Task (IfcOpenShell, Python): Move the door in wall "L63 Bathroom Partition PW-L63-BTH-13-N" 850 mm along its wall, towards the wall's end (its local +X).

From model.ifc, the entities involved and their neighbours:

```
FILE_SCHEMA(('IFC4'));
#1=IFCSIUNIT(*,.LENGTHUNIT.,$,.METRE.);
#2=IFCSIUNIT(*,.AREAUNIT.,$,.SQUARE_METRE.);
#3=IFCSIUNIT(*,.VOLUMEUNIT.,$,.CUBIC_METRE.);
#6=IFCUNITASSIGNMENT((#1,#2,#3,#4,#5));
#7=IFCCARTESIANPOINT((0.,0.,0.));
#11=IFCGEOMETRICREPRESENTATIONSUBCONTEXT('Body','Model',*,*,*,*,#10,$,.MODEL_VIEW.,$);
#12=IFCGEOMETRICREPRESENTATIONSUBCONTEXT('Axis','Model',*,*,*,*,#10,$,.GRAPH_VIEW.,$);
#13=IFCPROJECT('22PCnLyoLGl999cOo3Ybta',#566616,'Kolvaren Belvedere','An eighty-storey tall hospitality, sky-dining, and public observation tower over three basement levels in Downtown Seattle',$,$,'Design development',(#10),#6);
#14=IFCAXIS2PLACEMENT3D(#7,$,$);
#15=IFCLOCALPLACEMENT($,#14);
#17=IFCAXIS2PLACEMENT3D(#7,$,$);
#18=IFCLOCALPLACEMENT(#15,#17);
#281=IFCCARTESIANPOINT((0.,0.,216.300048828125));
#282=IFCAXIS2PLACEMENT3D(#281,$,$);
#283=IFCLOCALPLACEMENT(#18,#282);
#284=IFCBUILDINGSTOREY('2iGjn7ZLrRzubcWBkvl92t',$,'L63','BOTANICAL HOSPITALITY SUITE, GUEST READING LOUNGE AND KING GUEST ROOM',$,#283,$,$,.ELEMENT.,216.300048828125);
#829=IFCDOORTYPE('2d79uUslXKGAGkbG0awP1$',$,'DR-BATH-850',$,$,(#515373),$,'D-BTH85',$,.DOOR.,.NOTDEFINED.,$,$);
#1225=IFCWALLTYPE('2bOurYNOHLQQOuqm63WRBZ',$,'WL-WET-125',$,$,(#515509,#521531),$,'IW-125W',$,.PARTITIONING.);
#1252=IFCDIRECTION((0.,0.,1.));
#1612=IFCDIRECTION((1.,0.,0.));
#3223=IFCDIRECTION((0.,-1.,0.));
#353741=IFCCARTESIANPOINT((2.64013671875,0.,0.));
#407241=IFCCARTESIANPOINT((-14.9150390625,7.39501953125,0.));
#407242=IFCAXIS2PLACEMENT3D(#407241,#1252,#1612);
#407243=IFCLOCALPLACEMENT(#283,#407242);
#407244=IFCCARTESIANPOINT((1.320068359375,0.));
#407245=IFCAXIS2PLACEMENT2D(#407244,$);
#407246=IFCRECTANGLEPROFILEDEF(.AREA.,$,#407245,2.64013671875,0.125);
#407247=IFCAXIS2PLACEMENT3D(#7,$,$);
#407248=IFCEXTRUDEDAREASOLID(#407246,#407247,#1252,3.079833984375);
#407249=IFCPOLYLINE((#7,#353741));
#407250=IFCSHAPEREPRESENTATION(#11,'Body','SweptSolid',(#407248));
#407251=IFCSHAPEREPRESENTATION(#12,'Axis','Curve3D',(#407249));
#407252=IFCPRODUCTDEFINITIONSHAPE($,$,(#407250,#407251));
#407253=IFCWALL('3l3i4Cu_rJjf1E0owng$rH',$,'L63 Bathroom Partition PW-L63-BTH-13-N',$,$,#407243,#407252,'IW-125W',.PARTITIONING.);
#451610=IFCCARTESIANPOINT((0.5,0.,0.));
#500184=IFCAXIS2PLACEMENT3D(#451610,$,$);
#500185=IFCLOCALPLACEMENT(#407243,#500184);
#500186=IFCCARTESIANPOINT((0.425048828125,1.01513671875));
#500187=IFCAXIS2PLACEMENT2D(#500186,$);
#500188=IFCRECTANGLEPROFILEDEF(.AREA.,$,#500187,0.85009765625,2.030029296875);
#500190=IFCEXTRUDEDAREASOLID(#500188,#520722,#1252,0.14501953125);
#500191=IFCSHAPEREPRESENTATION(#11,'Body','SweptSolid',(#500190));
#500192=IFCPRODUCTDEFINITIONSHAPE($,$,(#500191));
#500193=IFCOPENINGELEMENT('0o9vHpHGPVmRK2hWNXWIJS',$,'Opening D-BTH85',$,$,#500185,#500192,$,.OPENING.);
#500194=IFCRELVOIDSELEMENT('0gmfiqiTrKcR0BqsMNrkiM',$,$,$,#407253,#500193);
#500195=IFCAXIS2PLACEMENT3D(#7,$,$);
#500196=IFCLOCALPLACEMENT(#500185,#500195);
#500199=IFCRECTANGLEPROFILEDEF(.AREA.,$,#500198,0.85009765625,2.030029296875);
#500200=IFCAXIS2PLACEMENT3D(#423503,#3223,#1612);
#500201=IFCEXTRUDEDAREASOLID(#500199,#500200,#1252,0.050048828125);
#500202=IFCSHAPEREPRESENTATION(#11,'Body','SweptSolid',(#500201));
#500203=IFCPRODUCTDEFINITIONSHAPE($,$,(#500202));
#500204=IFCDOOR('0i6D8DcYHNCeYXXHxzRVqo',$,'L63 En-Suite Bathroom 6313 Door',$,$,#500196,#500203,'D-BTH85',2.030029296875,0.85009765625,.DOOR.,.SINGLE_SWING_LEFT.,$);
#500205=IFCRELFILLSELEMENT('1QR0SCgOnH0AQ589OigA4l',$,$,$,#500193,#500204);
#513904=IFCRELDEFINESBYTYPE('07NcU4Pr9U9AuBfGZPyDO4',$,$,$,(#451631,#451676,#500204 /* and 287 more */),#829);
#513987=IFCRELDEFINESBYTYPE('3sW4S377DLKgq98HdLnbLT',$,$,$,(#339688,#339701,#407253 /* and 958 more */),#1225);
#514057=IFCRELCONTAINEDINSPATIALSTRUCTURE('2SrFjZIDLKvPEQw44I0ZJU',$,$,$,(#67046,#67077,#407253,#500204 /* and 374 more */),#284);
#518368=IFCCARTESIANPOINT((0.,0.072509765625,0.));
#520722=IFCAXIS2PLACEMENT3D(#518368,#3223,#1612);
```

```python
import ifcopenshell
import ifcopenshell.api.geometry
import ifcopenshell.util.placement
import ifcopenshell.util.unit

model = ifcopenshell.open("model.ifc")
unit_scale = ifcopenshell.util.unit.calculate_unit_scale(model)

door = model.by_guid("0i6D8DcYHNCeYXXHxzRVqo")
opening = door.FillsVoids[0].RelatingOpeningElement
wall = opening.VoidsElements[0].RelatingBuildingElement

wall_matrix = ifcopenshell.util.placement.get_local_placement(wall.ObjectPlacement)
shift = wall_matrix[:3, 0] * 0.85 / unit_scale
before = ifcopenshell.util.placement.get_local_placement(door.ObjectPlacement)[:3, 3].copy()

# The door is placed relative to its opening, so it follows when the opening moves.
matrix = ifcopenshell.util.placement.get_local_placement(opening.ObjectPlacement)
matrix[:3, 3] += shift
ifcopenshell.api.geometry.edit_object_placement(
    model, product=opening, matrix=matrix, is_si=False, should_transform_children=True
)

after = ifcopenshell.util.placement.get_local_placement(door.ObjectPlacement)[:3, 3]
print("door moved by", (after - before).round(3) + 0.0)

model.write("model_updated.ifc")
```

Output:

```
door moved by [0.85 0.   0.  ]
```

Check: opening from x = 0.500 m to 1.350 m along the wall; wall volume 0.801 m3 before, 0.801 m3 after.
